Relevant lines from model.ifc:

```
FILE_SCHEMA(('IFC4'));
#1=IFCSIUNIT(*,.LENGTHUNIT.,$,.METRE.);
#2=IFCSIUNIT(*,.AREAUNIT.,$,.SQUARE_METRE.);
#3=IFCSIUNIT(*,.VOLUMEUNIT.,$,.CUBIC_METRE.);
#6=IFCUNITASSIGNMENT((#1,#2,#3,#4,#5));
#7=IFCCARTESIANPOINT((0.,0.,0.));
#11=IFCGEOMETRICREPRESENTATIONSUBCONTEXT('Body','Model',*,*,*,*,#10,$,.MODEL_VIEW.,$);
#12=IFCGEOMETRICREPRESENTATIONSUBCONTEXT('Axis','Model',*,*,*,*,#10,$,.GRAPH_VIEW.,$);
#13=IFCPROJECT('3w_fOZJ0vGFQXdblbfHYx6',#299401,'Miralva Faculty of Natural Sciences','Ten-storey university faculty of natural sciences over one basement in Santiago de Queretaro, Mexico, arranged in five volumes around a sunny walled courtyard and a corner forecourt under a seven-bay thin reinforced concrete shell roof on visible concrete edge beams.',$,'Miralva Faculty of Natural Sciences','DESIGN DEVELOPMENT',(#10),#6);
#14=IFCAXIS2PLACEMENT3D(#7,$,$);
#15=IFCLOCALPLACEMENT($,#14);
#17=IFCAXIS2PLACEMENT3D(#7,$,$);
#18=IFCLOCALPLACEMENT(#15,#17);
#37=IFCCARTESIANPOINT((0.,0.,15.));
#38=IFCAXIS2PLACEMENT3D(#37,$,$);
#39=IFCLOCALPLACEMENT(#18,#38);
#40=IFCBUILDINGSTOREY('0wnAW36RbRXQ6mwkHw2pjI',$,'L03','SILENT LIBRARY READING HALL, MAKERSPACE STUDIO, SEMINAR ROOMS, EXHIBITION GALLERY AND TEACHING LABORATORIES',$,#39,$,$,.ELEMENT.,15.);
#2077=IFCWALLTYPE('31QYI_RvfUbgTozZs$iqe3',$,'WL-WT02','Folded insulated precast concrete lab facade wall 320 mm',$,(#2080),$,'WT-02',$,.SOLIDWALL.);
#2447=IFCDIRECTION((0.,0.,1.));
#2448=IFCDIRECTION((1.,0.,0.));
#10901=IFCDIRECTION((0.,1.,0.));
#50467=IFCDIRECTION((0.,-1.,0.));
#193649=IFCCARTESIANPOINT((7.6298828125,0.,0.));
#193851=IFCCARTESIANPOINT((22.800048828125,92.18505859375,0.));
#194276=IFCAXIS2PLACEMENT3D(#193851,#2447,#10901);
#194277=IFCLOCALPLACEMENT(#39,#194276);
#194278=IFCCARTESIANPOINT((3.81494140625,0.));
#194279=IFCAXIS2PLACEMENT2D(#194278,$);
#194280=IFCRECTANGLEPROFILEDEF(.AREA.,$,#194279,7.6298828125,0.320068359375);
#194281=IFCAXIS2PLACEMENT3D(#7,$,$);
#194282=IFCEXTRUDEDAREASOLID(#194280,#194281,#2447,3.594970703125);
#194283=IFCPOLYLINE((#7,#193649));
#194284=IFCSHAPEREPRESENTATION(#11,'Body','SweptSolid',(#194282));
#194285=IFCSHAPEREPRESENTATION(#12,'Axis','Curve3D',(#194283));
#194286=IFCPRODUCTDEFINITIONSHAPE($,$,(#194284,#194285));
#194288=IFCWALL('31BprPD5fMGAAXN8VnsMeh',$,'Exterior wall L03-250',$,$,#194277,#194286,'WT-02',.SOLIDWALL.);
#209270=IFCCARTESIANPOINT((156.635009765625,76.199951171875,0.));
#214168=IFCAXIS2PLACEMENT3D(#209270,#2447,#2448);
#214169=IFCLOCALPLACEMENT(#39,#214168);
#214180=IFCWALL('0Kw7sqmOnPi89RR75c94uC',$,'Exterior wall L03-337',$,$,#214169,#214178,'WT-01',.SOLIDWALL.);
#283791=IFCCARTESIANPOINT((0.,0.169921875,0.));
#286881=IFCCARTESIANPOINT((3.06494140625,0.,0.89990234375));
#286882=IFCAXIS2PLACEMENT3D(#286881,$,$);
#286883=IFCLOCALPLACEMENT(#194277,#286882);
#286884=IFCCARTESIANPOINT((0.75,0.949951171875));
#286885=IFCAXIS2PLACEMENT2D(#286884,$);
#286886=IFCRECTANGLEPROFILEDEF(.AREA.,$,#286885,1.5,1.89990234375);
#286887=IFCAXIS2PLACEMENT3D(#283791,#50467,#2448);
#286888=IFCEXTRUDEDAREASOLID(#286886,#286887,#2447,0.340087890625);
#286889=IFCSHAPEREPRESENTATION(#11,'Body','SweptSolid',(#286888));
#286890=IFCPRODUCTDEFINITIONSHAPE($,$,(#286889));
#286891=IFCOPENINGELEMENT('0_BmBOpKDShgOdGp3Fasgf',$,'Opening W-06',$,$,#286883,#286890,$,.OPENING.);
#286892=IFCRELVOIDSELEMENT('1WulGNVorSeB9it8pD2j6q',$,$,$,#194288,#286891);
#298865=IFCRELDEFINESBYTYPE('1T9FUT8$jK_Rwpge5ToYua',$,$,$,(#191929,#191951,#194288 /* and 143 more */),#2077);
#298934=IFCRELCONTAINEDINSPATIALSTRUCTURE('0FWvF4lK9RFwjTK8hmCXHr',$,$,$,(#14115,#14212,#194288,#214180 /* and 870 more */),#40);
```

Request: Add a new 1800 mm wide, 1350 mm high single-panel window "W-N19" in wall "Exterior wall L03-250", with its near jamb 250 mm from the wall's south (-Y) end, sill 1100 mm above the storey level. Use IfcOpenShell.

```python
import numpy as np
import ifcopenshell
import ifcopenshell.api.feature
import ifcopenshell.api.geometry
import ifcopenshell.api.root
import ifcopenshell.api.spatial
import ifcopenshell.geom
import ifcopenshell.util.element
import ifcopenshell.util.placement
import ifcopenshell.util.representation
import ifcopenshell.util.shape
import ifcopenshell.util.unit

model = ifcopenshell.open("model.ifc")
unit_scale = ifcopenshell.util.unit.calculate_unit_scale(model)
settings = ifcopenshell.geom.settings()


def volume(element):
    """Net volume in cubic metres, openings subtracted."""
    shape = ifcopenshell.geom.create_shape(settings, element)
    return ifcopenshell.util.shape.get_volume(shape.geometry)


wall = model.by_guid("31BprPD5fMGAAXN8VnsMeh")
storey = ifcopenshell.util.element.get_container(wall, ifc_class="IfcBuildingStorey")
context = ifcopenshell.util.representation.get_context(model, "Model", "Body", "MODEL_VIEW")
before = volume(wall)

width, height, from_end, sill = 1.8, 1.35, 0.25, 1.1  # metres

# The wall runs along its own X axis, and the end named is its -X end.
wall_shape = ifcopenshell.geom.create_shape(settings, wall)
x, y, z = ifcopenshell.util.shape.get_vertices(wall_shape.geometry).T
start = x.min() + from_end
face, thickness = float(y.min()), float(y.max() - y.min())
wall_matrix = ifcopenshell.util.placement.get_local_placement(wall.ObjectPlacement)
level = ifcopenshell.util.placement.get_local_placement(storey.ObjectPlacement)[2, 3]


def in_wall(x, y):
    """Placement at x, y metres in the wall's axes, at sill height."""
    matrix = wall_matrix.copy()
    matrix[:, 3] = wall_matrix @ np.array([x / unit_scale, y / unit_scale, 0.0, 1.0])
    matrix[2, 3] = level + sill / unit_scale
    return matrix


# Opening: a box that overshoots both wall faces by 50 mm.
opening = ifcopenshell.api.root.create_entity(model, ifc_class="IfcOpeningElement", predefined_type="OPENING")
box = ifcopenshell.api.geometry.add_wall_representation(
    model, context=context, length=width, height=height, thickness=thickness + 0.1
)
ifcopenshell.api.geometry.assign_representation(model, product=opening, representation=box)
ifcopenshell.api.geometry.edit_object_placement(model, product=opening, matrix=in_wall(start, face - 0.05), is_si=False)
ifcopenshell.api.feature.add_feature(model, feature=opening, element=wall)

window = ifcopenshell.api.root.create_entity(model, ifc_class="IfcWindow", name="W-N19", predefined_type="WINDOW")
window.OverallWidth, window.OverallHeight = width / unit_scale, height / unit_scale
window.PartitioningType = "SINGLE_PANEL"
body = ifcopenshell.api.geometry.add_window_representation(
    model,
    context=context,
    overall_width=window.OverallWidth,
    overall_height=window.OverallHeight,
    partition_type="SINGLE_PANEL",
)
ifcopenshell.api.geometry.assign_representation(model, product=window, representation=body)
ifcopenshell.api.spatial.assign_container(model, products=[window], relating_structure=storey)
ifcopenshell.api.feature.add_filling(model, opening=opening, element=window)

# Centre the window in the wall's thickness.
ifcopenshell.api.geometry.edit_object_placement(model, product=window, matrix=in_wall(start, face), is_si=False)
window_shape = ifcopenshell.geom.create_shape(settings, window)
depth = ifcopenshell.util.shape.get_vertices(window_shape.geometry)[:, 1]
offset = face + thickness / 2 - (depth.min() + depth.max()) / 2
ifcopenshell.api.geometry.edit_object_placement(model, product=window, matrix=in_wall(start, offset), is_si=False)

after = volume(wall)

print(f"wall volume {before:.3f} -> {after:.3f} m3")

model.write("model-out.ifc")
```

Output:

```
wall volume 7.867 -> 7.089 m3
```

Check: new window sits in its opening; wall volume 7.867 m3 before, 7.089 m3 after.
